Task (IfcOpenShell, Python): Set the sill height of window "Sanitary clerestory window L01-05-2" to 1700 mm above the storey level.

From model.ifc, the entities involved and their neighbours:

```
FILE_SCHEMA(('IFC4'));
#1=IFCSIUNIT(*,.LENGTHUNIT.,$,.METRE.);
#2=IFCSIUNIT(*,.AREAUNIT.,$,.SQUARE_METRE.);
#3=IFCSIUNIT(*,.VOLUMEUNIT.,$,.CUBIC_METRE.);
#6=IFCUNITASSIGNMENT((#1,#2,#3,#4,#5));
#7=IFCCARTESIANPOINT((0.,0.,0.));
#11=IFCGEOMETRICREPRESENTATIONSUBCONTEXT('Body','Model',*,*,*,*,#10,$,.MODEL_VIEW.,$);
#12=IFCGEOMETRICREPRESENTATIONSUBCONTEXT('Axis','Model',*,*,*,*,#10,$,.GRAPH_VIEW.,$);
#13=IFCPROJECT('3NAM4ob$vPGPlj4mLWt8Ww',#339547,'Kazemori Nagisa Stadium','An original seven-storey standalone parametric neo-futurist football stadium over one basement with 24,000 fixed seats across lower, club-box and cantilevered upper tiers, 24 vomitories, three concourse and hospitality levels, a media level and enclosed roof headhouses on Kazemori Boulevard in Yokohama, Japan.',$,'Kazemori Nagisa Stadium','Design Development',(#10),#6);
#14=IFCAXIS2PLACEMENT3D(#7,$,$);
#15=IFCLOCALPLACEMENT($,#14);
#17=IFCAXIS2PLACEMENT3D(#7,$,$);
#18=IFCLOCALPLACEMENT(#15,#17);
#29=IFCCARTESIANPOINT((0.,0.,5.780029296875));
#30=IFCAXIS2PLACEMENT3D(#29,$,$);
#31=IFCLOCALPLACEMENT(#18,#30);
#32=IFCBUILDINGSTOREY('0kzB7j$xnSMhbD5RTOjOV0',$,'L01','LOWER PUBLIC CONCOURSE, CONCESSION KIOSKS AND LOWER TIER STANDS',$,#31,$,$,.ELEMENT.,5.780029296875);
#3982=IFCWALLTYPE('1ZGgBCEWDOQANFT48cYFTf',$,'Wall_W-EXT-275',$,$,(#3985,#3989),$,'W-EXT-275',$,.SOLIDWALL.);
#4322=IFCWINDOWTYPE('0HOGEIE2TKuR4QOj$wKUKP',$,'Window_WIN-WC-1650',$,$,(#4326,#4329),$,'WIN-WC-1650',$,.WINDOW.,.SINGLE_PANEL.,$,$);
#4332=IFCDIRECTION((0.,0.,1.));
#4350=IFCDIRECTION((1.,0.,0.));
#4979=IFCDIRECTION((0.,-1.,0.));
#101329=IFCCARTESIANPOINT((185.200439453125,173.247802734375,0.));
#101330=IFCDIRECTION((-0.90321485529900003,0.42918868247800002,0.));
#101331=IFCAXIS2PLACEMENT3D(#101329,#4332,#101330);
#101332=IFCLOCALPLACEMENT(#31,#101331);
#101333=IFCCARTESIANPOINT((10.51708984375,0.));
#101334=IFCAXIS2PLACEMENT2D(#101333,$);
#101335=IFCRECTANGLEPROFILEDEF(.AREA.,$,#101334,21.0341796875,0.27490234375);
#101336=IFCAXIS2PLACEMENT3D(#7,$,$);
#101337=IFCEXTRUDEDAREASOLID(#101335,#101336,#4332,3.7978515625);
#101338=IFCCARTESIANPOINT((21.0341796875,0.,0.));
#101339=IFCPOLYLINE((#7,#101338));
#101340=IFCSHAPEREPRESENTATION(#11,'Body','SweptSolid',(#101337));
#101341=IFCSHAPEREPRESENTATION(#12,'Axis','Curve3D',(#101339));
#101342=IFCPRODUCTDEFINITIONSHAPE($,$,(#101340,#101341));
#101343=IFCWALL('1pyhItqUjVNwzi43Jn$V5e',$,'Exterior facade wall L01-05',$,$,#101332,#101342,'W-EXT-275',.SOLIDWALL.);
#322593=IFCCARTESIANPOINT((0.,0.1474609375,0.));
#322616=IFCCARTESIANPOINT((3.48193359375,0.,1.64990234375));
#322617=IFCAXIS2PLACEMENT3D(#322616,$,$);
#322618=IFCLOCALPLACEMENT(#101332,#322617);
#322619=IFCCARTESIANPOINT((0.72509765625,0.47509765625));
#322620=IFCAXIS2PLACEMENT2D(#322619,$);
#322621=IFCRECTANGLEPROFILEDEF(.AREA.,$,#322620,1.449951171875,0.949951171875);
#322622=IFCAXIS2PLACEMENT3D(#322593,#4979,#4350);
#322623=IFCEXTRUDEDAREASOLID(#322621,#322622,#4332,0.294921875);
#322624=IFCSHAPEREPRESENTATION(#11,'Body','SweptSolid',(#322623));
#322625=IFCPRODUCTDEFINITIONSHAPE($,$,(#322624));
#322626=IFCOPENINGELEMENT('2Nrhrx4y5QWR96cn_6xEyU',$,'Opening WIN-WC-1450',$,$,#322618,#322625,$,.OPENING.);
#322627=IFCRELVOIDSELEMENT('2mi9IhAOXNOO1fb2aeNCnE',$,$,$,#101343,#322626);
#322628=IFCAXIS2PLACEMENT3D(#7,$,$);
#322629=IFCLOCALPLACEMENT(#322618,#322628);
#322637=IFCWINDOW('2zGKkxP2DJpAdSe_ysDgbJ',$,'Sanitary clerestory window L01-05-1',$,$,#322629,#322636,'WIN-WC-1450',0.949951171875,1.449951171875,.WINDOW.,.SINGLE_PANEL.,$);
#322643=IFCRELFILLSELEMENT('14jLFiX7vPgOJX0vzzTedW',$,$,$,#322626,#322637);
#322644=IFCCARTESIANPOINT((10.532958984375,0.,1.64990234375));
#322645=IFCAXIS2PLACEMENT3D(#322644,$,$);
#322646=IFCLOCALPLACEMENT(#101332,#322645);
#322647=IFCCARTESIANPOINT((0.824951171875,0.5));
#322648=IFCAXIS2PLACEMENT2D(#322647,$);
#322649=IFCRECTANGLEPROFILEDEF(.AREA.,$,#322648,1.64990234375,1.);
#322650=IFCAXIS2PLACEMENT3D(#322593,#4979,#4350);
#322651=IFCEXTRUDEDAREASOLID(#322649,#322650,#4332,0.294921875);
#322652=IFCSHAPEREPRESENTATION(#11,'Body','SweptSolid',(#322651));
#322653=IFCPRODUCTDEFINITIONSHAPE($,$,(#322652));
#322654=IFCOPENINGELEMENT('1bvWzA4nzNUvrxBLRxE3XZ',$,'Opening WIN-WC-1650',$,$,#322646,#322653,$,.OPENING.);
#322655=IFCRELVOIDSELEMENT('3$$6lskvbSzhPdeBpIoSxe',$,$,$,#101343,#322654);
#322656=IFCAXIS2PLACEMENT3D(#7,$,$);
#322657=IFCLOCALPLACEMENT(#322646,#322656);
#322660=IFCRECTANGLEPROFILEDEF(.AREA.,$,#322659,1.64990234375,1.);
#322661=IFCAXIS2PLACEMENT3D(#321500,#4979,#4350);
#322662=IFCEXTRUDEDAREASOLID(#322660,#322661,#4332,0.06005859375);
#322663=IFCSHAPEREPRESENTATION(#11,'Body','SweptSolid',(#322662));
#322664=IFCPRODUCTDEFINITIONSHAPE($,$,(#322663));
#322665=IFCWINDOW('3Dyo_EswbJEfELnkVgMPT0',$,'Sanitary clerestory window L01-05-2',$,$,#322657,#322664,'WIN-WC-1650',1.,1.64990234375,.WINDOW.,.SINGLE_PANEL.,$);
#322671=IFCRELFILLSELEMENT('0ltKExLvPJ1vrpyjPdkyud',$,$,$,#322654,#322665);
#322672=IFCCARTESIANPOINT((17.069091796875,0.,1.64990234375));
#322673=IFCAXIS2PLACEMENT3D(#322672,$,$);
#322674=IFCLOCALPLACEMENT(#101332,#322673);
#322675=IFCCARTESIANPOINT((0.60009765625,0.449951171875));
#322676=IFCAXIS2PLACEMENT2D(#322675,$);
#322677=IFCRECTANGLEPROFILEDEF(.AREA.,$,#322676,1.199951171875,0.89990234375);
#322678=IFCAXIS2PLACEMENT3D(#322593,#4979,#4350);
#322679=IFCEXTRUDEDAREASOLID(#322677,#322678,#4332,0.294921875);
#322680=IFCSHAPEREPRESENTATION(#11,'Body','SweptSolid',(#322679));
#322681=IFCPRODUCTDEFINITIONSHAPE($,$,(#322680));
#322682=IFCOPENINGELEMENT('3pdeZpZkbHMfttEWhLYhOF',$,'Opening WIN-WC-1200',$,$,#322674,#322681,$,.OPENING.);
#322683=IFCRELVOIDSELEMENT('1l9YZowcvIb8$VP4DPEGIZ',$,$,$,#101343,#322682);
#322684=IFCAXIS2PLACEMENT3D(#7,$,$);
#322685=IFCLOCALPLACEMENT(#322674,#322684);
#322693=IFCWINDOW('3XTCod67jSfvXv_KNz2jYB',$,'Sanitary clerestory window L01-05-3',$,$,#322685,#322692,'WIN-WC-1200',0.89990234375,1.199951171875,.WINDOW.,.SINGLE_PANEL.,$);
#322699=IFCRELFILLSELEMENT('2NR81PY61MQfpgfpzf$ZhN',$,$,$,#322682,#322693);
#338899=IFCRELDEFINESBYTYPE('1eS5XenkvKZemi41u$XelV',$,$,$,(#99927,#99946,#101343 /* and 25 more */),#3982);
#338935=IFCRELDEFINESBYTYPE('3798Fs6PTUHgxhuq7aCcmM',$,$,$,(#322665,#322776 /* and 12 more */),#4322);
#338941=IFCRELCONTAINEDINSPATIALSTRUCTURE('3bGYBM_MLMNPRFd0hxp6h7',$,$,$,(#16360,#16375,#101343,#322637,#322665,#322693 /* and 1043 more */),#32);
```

```python
import numpy as np
import ifcopenshell
import ifcopenshell.api.geometry
import ifcopenshell.geom
import ifcopenshell.util.element
import ifcopenshell.util.placement
import ifcopenshell.util.shape
import ifcopenshell.util.unit

model = ifcopenshell.open("model.ifc")
unit_scale = ifcopenshell.util.unit.calculate_unit_scale(model)

window = model.by_guid("3Dyo_EswbJEfELnkVgMPT0")
opening = window.FillsVoids[0].RelatingOpeningElement
storey = ifcopenshell.util.element.get_container(window, ifc_class="IfcBuildingStorey")
level = ifcopenshell.util.placement.get_local_placement(storey.ObjectPlacement)[2, 3]

# The opening's origin need not be at the sill, so measure its lowest point.
shape = ifcopenshell.geom.create_shape(ifcopenshell.geom.settings(), opening)
bottom = ifcopenshell.util.shape.get_shape_bottom_elevation(shape, shape.geometry) / unit_scale
dz = level + 1.7 / unit_scale - bottom

shift = np.array([0.0, 0.0, dz])
# The window is placed relative to its opening, so it follows when the opening moves.
matrix = ifcopenshell.util.placement.get_local_placement(opening.ObjectPlacement)
matrix[:3, 3] += shift
ifcopenshell.api.geometry.edit_object_placement(
    model, product=opening, matrix=matrix, is_si=False, should_transform_children=True
)

print(f"moved by {dz * unit_scale:+.3f} m")

model.write("model-out.ifc")
```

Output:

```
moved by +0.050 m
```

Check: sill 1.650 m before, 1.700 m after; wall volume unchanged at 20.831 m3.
